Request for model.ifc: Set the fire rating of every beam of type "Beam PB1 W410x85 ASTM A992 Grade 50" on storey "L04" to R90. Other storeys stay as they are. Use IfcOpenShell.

First a look at what the model holds.

```python
import ifcopenshell
import ifcopenshell.util.element

model = ifcopenshell.open("model.ifc")
print(model.schema)
storey = next(s for s in model.by_type("IfcBuildingStorey") if s.Name == "L04")
beams = [e for e in ifcopenshell.util.element.get_decomposition(storey) if e.is_a("IfcBeam")]
seen = {}
for e in beams:
    element_type = ifcopenshell.util.element.get_type(e)
    key = (element_type.Name if element_type != e and element_type else None, ifcopenshell.util.element.get_pset(e, "Pset_BeamCommon", "FireRating"))
    seen[key] = seen.get(key, 0) + 1
for (name, value), count in sorted(seen.items(), key=str):
    print(count, "x", name, "|", value)
```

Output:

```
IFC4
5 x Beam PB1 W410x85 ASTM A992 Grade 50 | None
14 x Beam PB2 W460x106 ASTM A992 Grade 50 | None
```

```python
import ifcopenshell
import ifcopenshell.api.pset
import ifcopenshell.util.element

model = ifcopenshell.open("model.ifc")

storey = next(s for s in model.by_type("IfcBuildingStorey") if s.Name == "L04")
beams = [e for e in ifcopenshell.util.element.get_decomposition(storey) if e.is_a("IfcBeam")]

count = 0
for e in beams:
    element_type = ifcopenshell.util.element.get_type(e)
    if element_type in (None, e) or element_type.Name != "Beam PB1 W410x85 ASTM A992 Grade 50":
        continue
    found = ifcopenshell.util.element.get_pset(e, "Pset_BeamCommon", should_inherit=False)
    if found:
        pset = model.by_id(found["id"])
        if len(ifcopenshell.util.element.get_elements_by_pset(pset)) > 1:
            pset = ifcopenshell.api.pset.unshare_pset(model, products=[e], pset=pset)[0]
    else:
        pset = ifcopenshell.api.pset.add_pset(model, product=e, name="Pset_BeamCommon")
    ifcopenshell.api.pset.edit_pset(model, pset=pset, properties={"FireRating": "R90"})
    count += 1

print(count, "beams updated")

model.write("model_edited.ifc")
```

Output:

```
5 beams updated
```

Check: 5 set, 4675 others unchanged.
